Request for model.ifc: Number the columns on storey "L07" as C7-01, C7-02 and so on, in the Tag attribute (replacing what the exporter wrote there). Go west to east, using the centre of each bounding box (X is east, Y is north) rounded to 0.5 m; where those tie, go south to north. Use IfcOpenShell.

First a look at what the model holds.

```python
import ifcopenshell
import ifcopenshell.util.element
import ifcopenshell.util.placement

model = ifcopenshell.open("model.ifc")
print(model.schema)
storey = next(s for s in model.by_type("IfcBuildingStorey") if s.Name == "L07")
columns = [e for e in ifcopenshell.util.element.get_decomposition(storey) if e.is_a("IfcColumn")]
for e in sorted(columns, key=lambda e: e.id()):
    origin = ifcopenshell.util.placement.get_local_placement(e.ObjectPlacement)[:3, 3]
    print(e.id(), e.Tag, e.Name, origin.round(2) + 0.0, sep=" | ")
```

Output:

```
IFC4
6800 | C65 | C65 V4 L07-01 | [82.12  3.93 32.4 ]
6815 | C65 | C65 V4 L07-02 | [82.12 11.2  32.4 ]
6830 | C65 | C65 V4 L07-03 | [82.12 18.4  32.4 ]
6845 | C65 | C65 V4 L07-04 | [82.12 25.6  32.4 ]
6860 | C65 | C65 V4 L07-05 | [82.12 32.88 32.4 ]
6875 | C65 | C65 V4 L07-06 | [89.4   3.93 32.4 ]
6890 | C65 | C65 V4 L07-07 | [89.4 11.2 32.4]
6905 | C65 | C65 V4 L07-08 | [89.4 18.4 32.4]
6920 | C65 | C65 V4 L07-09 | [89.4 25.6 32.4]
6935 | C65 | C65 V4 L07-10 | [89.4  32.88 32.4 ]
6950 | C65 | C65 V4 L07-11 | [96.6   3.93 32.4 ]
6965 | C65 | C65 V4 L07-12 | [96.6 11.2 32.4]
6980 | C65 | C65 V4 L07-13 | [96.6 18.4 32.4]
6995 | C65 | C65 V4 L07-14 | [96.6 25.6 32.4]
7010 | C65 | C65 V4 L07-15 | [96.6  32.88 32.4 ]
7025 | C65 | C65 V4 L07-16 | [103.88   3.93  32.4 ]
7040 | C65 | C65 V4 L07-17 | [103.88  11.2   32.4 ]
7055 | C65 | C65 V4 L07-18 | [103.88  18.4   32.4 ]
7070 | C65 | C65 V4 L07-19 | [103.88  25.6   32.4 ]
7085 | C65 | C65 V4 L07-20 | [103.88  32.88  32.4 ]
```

```python
import ifcopenshell
import ifcopenshell.geom
import ifcopenshell.util.element
import ifcopenshell.util.shape

model = ifcopenshell.open("model.ifc")
settings = ifcopenshell.geom.settings()
settings.set("use-world-coords", True)


def centre(element):
    shape = ifcopenshell.geom.create_shape(settings, element)
    return ifcopenshell.util.shape.get_bbox_centroid(shape.geometry)


storey = next(s for s in model.by_type("IfcBuildingStorey") if s.Name == "L07")
columns = [e for e in ifcopenshell.util.element.get_decomposition(storey) if e.is_a("IfcColumn")]

# Insertion points can sit at a corner or the storey origin, so sort by the geometry (in metres).
centres = {e: centre(e) for e in columns}
columns.sort(key=lambda e: (round(centres[e][0] / 0.5), centres[e][1]))

for i, e in enumerate(columns, start=1):
    number = f"C7-{i:02d}"
    e.Tag = number
    print(e.id(), number)

model.write("model_v2.ifc")
```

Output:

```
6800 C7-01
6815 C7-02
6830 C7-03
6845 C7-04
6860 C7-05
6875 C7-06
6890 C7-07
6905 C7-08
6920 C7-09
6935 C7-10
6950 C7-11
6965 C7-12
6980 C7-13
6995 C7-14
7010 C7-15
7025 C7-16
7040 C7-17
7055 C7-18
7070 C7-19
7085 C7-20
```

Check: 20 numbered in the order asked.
